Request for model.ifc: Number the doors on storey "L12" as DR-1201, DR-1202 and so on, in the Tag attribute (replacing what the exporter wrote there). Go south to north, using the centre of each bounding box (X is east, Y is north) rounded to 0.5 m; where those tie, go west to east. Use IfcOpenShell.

First a look at what the model holds.

```python
import ifcopenshell
import ifcopenshell.util.element
import ifcopenshell.util.placement

model = ifcopenshell.open("model.ifc")
print(model.schema)
storey = next(s for s in model.by_type("IfcBuildingStorey") if s.Name == "L12")
doors = [e for e in ifcopenshell.util.element.get_decomposition(storey) if e.is_a("IfcDoor")]
for e in sorted(doors, key=lambda e: e.id()):
    origin = ifcopenshell.util.placement.get_local_placement(e.ObjectPlacement)[:3, 3]
    print(e.id(), e.Tag, e.Name, origin.round(2) + 0.0, sep=" | ")
```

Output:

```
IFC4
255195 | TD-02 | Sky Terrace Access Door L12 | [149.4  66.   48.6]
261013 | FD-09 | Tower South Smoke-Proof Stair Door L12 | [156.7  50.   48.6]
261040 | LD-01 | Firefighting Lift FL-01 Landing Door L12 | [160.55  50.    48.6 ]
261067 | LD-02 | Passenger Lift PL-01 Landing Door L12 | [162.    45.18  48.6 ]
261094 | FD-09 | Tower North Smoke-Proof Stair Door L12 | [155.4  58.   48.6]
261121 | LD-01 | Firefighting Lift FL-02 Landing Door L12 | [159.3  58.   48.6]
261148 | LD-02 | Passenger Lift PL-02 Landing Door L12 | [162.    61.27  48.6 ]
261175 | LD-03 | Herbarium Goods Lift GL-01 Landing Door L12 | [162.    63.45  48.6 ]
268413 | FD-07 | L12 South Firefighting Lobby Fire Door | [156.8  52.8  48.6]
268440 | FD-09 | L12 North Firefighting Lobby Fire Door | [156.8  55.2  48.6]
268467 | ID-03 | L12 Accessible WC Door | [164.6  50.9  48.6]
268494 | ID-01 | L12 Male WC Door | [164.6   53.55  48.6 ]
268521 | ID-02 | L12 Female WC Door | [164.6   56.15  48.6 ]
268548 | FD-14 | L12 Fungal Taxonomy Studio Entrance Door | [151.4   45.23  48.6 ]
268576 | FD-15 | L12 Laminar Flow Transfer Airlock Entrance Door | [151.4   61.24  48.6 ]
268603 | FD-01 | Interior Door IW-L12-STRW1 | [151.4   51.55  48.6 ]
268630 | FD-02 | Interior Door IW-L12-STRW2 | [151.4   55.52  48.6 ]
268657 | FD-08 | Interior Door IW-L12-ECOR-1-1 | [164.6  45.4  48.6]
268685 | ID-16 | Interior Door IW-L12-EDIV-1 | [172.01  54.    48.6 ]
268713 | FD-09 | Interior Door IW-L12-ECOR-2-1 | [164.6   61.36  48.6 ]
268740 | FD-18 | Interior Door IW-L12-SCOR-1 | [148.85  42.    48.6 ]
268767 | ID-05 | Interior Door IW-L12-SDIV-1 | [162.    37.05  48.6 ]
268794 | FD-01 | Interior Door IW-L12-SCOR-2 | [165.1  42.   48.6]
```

```python
import ifcopenshell
import ifcopenshell.geom
import ifcopenshell.util.element
import ifcopenshell.util.shape

model = ifcopenshell.open("model.ifc")
settings = ifcopenshell.geom.settings()
settings.set("use-world-coords", True)


def centre(element):
    shape = ifcopenshell.geom.create_shape(settings, element)
    return ifcopenshell.util.shape.get_bbox_centroid(shape.geometry)


storey = next(s for s in model.by_type("IfcBuildingStorey") if s.Name == "L12")
doors = [e for e in ifcopenshell.util.element.get_decomposition(storey) if e.is_a("IfcDoor")]

# Insertion points can sit at a corner or the storey origin, so sort by the geometry (in metres).
centres = {e: centre(e) for e in doors}
doors.sort(key=lambda e: (round(centres[e][1] / 0.5), centres[e][0]))

for i, e in enumerate(doors, start=1):
    number = f"DR-12{i:02d}"
    e.Tag = number
    print(e.id(), number)

model.write("model_updated.ifc")
```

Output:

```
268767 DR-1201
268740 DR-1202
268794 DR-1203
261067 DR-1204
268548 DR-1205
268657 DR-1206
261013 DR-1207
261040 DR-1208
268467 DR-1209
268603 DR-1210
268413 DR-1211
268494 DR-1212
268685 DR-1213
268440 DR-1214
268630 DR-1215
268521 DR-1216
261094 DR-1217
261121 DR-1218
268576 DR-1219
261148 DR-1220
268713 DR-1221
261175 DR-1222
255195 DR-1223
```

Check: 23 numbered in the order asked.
